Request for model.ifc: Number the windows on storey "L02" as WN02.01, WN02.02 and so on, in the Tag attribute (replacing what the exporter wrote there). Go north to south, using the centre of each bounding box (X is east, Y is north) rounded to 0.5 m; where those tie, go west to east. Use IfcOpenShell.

First a look at what the model holds.

```python
import ifcopenshell
import ifcopenshell.util.element
import ifcopenshell.util.placement

model = ifcopenshell.open("model.ifc")
print(model.schema)
storey = next(s for s in model.by_type("IfcBuildingStorey") if s.Name == "L02")
windows = [e for e in ifcopenshell.util.element.get_decomposition(storey) if e.is_a("IfcWindow")]
for e in sorted(windows, key=lambda e: e.id()):
    origin = ifcopenshell.util.placement.get_local_placement(e.ObjectPlacement)[:3, 3]
    print(e.id(), e.Tag, e.Name, origin.round(2) + 0.0, sep=" | ")
```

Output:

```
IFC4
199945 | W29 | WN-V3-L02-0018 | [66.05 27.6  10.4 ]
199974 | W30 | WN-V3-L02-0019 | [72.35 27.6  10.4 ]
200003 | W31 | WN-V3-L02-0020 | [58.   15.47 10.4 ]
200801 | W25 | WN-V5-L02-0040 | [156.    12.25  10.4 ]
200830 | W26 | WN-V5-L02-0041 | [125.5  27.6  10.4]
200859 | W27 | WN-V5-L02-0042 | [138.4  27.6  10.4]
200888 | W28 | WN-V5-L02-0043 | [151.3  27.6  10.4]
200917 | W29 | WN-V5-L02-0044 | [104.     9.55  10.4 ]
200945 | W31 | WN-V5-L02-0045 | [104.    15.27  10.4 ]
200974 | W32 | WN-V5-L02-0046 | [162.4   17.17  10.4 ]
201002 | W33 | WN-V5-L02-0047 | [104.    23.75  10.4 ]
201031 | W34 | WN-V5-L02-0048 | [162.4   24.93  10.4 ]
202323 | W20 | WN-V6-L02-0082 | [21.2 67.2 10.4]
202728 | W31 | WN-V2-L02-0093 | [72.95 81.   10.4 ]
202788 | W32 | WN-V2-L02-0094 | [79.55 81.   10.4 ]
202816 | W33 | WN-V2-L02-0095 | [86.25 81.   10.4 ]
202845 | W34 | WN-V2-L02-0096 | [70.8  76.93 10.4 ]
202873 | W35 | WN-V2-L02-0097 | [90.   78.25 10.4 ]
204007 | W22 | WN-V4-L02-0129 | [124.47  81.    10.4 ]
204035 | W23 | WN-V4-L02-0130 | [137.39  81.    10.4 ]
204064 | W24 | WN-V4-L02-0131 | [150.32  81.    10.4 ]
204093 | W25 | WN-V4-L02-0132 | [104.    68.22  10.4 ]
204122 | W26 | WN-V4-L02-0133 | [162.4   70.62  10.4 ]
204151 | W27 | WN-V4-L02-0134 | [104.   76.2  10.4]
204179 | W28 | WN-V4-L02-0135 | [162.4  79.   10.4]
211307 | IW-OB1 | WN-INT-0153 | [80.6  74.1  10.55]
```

```python
import ifcopenshell
import ifcopenshell.geom
import ifcopenshell.util.element
import ifcopenshell.util.shape

model = ifcopenshell.open("model.ifc")
settings = ifcopenshell.geom.settings()
settings.set("use-world-coords", True)


def centre(element):
    shape = ifcopenshell.geom.create_shape(settings, element)
    return ifcopenshell.util.shape.get_bbox_centroid(shape.geometry)


storey = next(s for s in model.by_type("IfcBuildingStorey") if s.Name == "L02")
windows = [e for e in ifcopenshell.util.element.get_decomposition(storey) if e.is_a("IfcWindow")]

# Insertion points can sit at a corner or the storey origin, so sort by the geometry (in metres).
centres = {e: centre(e) for e in windows}
windows.sort(key=lambda e: (-round(centres[e][1] / 0.5), centres[e][0]))

for i, e in enumerate(windows, start=1):
    number = f"WN02.{i:02d}"
    e.Tag = number
    print(e.id(), number)

model.write("model_v2.ifc")
```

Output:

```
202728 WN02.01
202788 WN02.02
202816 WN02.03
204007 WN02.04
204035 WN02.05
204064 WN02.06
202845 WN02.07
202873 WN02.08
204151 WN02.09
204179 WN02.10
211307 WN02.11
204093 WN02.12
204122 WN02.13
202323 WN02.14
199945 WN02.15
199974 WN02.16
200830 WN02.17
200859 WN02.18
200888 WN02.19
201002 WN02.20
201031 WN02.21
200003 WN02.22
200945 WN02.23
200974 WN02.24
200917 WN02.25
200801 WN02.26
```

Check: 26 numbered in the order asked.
